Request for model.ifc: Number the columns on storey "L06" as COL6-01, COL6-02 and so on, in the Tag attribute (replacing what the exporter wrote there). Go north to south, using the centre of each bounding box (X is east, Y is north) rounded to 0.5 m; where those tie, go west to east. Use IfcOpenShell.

First a look at what the model holds.

```python
import ifcopenshell
import ifcopenshell.util.element
import ifcopenshell.util.placement

model = ifcopenshell.open("model.ifc")
print(model.schema)
storey = next(s for s in model.by_type("IfcBuildingStorey") if s.Name == "L06")
columns = [e for e in ifcopenshell.util.element.get_decomposition(storey) if e.is_a("IfcColumn")]
for e in sorted(columns, key=lambda e: e.id()):
    origin = ifcopenshell.util.placement.get_local_placement(e.ObjectPlacement)[:3, 3]
    print(e.id(), e.Tag, e.Name, origin.round(2) + 0.0, sep=" | ")
```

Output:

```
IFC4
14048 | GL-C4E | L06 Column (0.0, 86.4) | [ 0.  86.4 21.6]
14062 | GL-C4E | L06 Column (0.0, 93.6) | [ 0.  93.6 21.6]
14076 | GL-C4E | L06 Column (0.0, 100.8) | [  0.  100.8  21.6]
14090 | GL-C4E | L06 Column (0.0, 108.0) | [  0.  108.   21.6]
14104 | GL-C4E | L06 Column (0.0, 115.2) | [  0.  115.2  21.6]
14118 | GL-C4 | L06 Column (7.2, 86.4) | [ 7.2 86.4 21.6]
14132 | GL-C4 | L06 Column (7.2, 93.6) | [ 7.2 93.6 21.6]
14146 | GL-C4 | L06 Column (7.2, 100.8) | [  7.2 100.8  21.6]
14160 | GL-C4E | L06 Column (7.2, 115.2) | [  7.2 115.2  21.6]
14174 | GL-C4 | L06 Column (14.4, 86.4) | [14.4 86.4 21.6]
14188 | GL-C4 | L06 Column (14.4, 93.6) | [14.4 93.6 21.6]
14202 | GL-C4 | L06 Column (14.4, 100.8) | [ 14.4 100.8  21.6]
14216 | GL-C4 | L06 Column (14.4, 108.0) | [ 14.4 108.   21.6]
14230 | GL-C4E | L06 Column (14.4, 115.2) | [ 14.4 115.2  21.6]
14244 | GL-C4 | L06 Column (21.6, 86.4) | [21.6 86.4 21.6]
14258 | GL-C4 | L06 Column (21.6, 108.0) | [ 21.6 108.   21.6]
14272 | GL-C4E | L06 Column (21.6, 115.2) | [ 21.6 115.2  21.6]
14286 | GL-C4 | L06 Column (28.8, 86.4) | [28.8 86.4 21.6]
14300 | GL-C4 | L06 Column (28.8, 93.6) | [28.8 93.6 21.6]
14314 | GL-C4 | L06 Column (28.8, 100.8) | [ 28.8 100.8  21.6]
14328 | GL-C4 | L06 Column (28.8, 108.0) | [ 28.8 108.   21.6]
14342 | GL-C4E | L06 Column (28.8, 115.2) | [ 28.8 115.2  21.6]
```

```python
import ifcopenshell
import ifcopenshell.geom
import ifcopenshell.util.element
import ifcopenshell.util.shape

model = ifcopenshell.open("model.ifc")
settings = ifcopenshell.geom.settings()
settings.set("use-world-coords", True)


def centre(element):
    shape = ifcopenshell.geom.create_shape(settings, element)
    return ifcopenshell.util.shape.get_bbox_centroid(shape.geometry)


storey = next(s for s in model.by_type("IfcBuildingStorey") if s.Name == "L06")
columns = [e for e in ifcopenshell.util.element.get_decomposition(storey) if e.is_a("IfcColumn")]

# Insertion points can sit at a corner or the storey origin, so sort by the geometry (in metres).
centres = {e: centre(e) for e in columns}
columns.sort(key=lambda e: (-round(centres[e][1] / 0.5), centres[e][0]))

for i, e in enumerate(columns, start=1):
    number = f"COL6-{i:02d}"
    e.Tag = number
    print(e.id(), number)

model.write("model_edited.ifc")
```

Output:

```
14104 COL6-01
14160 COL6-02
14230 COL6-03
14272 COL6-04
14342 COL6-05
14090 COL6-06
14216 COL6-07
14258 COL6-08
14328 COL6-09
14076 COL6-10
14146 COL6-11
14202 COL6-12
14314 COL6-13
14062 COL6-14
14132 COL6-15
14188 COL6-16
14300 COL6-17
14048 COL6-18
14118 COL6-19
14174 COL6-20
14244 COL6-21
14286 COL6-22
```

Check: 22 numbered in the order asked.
